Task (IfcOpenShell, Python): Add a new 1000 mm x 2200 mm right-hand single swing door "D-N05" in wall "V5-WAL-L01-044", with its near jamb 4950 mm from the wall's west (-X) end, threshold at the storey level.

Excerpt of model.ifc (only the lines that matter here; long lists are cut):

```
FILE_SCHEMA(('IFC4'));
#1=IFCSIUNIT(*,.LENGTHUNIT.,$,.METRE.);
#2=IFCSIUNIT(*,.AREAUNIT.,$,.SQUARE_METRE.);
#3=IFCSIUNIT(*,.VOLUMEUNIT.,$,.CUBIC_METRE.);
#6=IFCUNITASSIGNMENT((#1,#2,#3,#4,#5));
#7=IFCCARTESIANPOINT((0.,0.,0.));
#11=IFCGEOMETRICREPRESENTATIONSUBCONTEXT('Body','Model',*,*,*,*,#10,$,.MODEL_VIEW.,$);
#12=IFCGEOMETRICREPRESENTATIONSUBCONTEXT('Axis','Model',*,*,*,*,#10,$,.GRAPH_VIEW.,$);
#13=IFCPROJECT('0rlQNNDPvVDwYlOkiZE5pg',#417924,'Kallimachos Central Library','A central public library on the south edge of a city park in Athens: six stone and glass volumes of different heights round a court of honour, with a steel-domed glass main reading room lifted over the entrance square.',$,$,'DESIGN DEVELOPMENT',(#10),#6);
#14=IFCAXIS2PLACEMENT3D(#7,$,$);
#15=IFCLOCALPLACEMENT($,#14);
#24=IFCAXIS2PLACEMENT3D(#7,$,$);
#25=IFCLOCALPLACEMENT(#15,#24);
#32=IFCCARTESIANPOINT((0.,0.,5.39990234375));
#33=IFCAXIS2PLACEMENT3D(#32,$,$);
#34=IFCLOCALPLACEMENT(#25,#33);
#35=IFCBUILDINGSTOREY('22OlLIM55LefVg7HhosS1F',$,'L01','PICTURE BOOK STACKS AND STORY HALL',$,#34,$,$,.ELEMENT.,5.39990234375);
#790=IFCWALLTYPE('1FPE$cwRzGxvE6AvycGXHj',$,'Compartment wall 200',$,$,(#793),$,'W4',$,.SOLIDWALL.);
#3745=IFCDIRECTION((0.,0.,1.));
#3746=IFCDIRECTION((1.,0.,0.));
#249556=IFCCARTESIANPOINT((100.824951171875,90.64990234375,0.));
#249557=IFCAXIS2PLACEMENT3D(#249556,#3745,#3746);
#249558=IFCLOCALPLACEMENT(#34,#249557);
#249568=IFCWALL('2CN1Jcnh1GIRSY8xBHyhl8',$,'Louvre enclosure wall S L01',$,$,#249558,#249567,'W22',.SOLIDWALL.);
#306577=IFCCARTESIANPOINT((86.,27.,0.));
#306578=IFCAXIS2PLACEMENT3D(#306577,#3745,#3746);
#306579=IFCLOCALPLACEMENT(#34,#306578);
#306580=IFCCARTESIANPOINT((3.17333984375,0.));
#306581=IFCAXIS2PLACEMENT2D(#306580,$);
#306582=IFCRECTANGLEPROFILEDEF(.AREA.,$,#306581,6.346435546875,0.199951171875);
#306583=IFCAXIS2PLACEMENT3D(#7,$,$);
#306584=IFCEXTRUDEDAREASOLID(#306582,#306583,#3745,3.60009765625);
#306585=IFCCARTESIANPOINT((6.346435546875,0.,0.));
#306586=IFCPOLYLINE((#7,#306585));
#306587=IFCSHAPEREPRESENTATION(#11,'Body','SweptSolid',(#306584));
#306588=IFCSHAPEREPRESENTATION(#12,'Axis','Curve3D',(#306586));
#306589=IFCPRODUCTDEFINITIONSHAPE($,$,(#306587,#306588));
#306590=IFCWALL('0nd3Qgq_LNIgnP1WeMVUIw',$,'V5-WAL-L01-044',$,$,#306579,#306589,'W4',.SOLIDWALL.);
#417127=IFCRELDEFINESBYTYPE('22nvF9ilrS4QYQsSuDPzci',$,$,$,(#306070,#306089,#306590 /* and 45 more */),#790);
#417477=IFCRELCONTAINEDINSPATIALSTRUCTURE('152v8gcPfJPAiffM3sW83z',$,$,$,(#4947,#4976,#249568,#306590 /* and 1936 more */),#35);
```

```python
import numpy as np
import ifcopenshell
import ifcopenshell.api.feature
import ifcopenshell.api.geometry
import ifcopenshell.api.root
import ifcopenshell.api.spatial
import ifcopenshell.geom
import ifcopenshell.util.element
import ifcopenshell.util.placement
import ifcopenshell.util.representation
import ifcopenshell.util.shape
import ifcopenshell.util.unit

model = ifcopenshell.open("model.ifc")
unit_scale = ifcopenshell.util.unit.calculate_unit_scale(model)
settings = ifcopenshell.geom.settings()


def volume(element):
    """Net volume in cubic metres, openings subtracted."""
    shape = ifcopenshell.geom.create_shape(settings, element)
    return ifcopenshell.util.shape.get_volume(shape.geometry)


wall = model.by_id(306590)
storey = ifcopenshell.util.element.get_container(wall, ifc_class="IfcBuildingStorey")
context = ifcopenshell.util.representation.get_context(model, "Model", "Body", "MODEL_VIEW")
before = volume(wall)

width, height, from_end, sill = 1, 2.2, 4.95, 0.0  # metres

# The wall runs along its own X axis, and the end named is its -X end.
wall_shape = ifcopenshell.geom.create_shape(settings, wall)
x, y, z = ifcopenshell.util.shape.get_vertices(wall_shape.geometry).T
start = x.min() + from_end
face, thickness = float(y.min()), float(y.max() - y.min())
wall_matrix = ifcopenshell.util.placement.get_local_placement(wall.ObjectPlacement)
level = ifcopenshell.util.placement.get_local_placement(storey.ObjectPlacement)[2, 3]


def in_wall(x, y):
    """Placement at x, y metres in the wall's axes, at sill height."""
    matrix = wall_matrix.copy()
    matrix[:, 3] = wall_matrix @ np.array([x / unit_scale, y / unit_scale, 0.0, 1.0])
    matrix[2, 3] = level + sill / unit_scale
    return matrix


# Opening: a box that overshoots both wall faces by 50 mm.
opening = ifcopenshell.api.root.create_entity(model, ifc_class="IfcOpeningElement", predefined_type="OPENING")
box = ifcopenshell.api.geometry.add_wall_representation(
    model, context=context, length=width, height=height, thickness=thickness + 0.1
)
ifcopenshell.api.geometry.assign_representation(model, product=opening, representation=box)
ifcopenshell.api.geometry.edit_object_placement(model, product=opening, matrix=in_wall(start, face - 0.05), is_si=False)
ifcopenshell.api.feature.add_feature(model, feature=opening, element=wall)

door = ifcopenshell.api.root.create_entity(model, ifc_class="IfcDoor", name="D-N05", predefined_type="DOOR")
door.OverallWidth, door.OverallHeight = width / unit_scale, height / unit_scale
door.OperationType = "SINGLE_SWING_RIGHT"
body = ifcopenshell.api.geometry.add_door_representation(
    model,
    context=context,
    overall_width=door.OverallWidth,
    overall_height=door.OverallHeight,
    operation_type="SINGLE_SWING_RIGHT",
    lining_properties={"LiningDepth": thickness / unit_scale, "ThresholdDepth": thickness / unit_scale},
)
ifcopenshell.api.geometry.assign_representation(model, product=door, representation=body)
ifcopenshell.api.spatial.assign_container(model, products=[door], relating_structure=storey)
ifcopenshell.api.feature.add_filling(model, opening=opening, element=door)

# The lining spans the wall, so the door starts at the wall face.
ifcopenshell.api.geometry.edit_object_placement(model, product=door, matrix=in_wall(start, face), is_si=False)

after = volume(wall)

print(f"wall volume {before:.3f} -> {after:.3f} m3")

model.write("model_updated.ifc")
```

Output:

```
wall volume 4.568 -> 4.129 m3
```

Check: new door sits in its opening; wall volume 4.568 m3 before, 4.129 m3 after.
